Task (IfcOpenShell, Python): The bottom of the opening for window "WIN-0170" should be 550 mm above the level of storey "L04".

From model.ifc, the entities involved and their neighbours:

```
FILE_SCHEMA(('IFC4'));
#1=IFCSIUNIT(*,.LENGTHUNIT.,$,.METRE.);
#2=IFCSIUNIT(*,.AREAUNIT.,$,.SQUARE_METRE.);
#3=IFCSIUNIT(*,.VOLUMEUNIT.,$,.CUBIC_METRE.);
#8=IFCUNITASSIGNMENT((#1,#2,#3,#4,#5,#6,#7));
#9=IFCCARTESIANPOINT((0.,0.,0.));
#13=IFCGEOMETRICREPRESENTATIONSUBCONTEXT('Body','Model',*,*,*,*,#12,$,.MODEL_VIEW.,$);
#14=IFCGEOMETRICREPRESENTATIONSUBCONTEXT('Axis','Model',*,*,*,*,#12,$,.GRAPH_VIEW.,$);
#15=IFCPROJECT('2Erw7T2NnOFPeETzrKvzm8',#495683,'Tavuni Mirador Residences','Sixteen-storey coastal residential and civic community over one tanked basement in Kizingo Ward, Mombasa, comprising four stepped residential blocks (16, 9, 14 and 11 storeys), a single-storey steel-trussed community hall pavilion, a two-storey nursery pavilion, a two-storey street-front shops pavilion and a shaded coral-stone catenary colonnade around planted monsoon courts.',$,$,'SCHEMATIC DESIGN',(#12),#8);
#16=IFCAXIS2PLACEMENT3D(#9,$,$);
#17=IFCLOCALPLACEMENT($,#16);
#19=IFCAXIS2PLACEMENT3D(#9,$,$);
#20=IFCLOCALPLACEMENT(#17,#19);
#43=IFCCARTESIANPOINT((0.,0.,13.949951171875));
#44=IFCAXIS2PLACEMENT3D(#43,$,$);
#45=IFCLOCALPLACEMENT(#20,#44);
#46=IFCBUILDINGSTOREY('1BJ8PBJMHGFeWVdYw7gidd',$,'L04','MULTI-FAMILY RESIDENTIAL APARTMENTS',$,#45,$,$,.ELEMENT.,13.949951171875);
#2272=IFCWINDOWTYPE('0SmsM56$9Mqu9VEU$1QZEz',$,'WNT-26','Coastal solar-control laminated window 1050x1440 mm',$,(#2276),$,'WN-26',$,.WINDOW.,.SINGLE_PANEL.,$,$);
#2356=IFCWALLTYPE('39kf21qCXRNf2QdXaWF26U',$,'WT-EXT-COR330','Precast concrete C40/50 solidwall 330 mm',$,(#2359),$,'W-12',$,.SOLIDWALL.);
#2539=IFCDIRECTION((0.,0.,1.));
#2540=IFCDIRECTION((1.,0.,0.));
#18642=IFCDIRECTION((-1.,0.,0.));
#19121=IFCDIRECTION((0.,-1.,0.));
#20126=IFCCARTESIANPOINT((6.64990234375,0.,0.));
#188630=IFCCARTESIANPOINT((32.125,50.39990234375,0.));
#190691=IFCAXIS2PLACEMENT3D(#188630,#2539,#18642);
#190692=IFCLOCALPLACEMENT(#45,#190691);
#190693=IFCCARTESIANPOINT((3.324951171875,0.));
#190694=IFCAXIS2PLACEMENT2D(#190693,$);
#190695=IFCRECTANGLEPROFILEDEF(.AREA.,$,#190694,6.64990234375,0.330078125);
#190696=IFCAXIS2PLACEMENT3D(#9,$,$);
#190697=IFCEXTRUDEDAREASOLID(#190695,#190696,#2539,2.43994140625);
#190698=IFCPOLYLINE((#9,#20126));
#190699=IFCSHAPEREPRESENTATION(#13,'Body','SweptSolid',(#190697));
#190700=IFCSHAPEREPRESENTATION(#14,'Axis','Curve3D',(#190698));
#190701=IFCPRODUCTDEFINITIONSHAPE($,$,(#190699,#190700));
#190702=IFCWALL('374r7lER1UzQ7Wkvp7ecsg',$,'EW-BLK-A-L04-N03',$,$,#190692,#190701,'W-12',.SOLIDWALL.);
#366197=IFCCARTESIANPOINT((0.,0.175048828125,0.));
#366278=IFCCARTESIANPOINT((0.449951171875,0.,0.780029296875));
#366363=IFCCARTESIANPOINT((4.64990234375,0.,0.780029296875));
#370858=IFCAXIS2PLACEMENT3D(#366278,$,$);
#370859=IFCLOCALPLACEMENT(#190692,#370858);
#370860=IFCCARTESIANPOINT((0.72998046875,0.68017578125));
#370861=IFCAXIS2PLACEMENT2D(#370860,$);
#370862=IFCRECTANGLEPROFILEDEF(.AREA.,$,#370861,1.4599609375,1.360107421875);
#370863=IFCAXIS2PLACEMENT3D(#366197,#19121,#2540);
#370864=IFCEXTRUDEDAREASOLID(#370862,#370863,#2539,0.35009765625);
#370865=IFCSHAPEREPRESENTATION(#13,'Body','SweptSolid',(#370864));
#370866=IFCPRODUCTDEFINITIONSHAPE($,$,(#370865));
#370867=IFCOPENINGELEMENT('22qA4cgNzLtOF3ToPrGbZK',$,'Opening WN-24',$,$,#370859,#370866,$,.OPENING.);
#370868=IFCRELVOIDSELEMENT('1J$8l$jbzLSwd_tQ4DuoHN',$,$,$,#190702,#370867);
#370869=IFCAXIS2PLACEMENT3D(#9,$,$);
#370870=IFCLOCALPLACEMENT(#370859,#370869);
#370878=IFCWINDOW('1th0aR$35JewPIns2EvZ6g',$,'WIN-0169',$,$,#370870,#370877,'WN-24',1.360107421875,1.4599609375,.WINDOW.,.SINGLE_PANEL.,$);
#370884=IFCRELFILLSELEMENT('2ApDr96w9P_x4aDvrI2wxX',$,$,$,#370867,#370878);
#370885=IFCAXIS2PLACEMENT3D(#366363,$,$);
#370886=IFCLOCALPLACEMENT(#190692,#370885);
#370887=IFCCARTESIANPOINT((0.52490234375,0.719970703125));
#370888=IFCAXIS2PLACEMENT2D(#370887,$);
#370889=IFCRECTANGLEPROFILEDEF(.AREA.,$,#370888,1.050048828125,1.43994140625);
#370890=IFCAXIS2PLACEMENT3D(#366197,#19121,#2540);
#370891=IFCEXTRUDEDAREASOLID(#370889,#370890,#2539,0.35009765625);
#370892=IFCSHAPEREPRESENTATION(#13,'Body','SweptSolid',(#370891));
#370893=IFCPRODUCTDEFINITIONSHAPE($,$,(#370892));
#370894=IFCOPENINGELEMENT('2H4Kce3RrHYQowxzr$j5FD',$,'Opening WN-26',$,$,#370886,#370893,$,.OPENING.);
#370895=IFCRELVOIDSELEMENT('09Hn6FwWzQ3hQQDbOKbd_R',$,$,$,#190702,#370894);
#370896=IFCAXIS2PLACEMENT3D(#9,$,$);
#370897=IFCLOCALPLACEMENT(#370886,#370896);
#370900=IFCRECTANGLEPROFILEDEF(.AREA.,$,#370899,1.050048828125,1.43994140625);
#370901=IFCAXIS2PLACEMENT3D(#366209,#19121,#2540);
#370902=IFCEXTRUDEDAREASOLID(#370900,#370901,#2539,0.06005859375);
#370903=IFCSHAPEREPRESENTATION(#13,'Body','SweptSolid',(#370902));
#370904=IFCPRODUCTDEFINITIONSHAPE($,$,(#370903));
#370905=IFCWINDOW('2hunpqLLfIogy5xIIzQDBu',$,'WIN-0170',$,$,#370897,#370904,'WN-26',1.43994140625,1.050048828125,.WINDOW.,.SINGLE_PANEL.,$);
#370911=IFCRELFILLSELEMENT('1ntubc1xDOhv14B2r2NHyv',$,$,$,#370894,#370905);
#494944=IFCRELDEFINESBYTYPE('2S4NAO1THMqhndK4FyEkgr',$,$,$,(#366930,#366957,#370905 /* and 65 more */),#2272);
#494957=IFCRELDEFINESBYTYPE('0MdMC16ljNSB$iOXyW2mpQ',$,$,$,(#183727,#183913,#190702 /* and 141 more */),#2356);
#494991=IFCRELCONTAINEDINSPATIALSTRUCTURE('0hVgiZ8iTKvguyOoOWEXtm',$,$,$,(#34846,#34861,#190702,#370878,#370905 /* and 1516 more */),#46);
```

```python
import numpy as np
import ifcopenshell
import ifcopenshell.api.geometry
import ifcopenshell.geom
import ifcopenshell.util.element
import ifcopenshell.util.placement
import ifcopenshell.util.shape
import ifcopenshell.util.unit

model = ifcopenshell.open("model.ifc")
unit_scale = ifcopenshell.util.unit.calculate_unit_scale(model)

window = model.by_guid("2hunpqLLfIogy5xIIzQDBu")
opening = window.FillsVoids[0].RelatingOpeningElement
storey = ifcopenshell.util.element.get_container(window, ifc_class="IfcBuildingStorey")
level = ifcopenshell.util.placement.get_local_placement(storey.ObjectPlacement)[2, 3]

# The opening's origin need not be at the sill, so measure its lowest point.
shape = ifcopenshell.geom.create_shape(ifcopenshell.geom.settings(), opening)
bottom = ifcopenshell.util.shape.get_shape_bottom_elevation(shape, shape.geometry) / unit_scale
dz = level + 0.55 / unit_scale - bottom

shift = np.array([0.0, 0.0, dz])
# The window is placed relative to its opening, so it follows when the opening moves.
matrix = ifcopenshell.util.placement.get_local_placement(opening.ObjectPlacement)
matrix[:3, 3] += shift
ifcopenshell.api.geometry.edit_object_placement(
    model, product=opening, matrix=matrix, is_si=False, should_transform_children=True
)

print(f"moved by {dz * unit_scale:+.3f} m")

model.write("model_rev.ifc")
```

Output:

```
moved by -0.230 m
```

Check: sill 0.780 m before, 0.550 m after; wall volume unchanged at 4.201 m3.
